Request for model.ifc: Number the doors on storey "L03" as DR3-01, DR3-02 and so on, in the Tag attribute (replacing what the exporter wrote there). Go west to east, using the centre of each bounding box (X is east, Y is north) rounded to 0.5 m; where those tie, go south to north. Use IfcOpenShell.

First a look at what the model holds.

```python
import ifcopenshell
import ifcopenshell.util.element
import ifcopenshell.util.placement

model = ifcopenshell.open("model.ifc")
print(model.schema)
storey = next(s for s in model.by_type("IfcBuildingStorey") if s.Name == "L03")
doors = [e for e in ifcopenshell.util.element.get_decomposition(storey) if e.is_a("IfcDoor")]
for e in sorted(doors, key=lambda e: e.id()):
    origin = ifcopenshell.util.placement.get_local_placement(e.ObjectPlacement)[:3, 3]
    print(e.id(), e.Tag, e.Name, origin.round(2) + 0.0, sep=" | ")
```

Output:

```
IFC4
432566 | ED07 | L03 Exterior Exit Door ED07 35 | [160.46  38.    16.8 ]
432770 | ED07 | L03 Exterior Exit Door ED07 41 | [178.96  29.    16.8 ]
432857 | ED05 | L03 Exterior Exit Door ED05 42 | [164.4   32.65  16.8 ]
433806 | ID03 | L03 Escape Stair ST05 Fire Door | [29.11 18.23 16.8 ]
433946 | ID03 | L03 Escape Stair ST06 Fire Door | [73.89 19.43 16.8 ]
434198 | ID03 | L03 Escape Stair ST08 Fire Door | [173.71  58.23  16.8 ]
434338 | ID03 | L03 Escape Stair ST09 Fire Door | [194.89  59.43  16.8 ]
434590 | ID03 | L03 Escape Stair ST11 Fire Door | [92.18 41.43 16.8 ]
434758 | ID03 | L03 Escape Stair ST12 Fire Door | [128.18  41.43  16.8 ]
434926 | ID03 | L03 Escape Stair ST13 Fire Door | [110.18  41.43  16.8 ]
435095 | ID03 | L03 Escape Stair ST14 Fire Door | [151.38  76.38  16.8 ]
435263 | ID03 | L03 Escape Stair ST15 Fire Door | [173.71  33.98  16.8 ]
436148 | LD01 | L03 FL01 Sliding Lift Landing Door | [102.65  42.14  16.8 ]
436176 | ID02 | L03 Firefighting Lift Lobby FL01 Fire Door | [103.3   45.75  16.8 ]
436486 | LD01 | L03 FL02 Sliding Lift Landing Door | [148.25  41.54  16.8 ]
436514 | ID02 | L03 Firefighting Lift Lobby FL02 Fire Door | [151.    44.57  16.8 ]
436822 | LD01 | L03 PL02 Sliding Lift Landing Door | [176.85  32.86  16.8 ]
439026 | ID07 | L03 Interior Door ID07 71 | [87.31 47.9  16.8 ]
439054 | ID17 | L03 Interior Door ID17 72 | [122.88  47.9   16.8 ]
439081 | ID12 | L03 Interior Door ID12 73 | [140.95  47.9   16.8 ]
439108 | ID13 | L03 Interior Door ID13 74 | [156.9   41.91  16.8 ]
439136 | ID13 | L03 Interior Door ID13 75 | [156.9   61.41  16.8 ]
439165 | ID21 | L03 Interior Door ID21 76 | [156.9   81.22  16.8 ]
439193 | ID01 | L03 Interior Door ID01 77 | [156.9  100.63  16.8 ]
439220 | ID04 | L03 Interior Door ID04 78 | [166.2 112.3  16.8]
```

```python
import ifcopenshell
import ifcopenshell.geom
import ifcopenshell.util.element
import ifcopenshell.util.shape

model = ifcopenshell.open("model.ifc")
settings = ifcopenshell.geom.settings()
settings.set("use-world-coords", True)


def centre(element):
    shape = ifcopenshell.geom.create_shape(settings, element)
    return ifcopenshell.util.shape.get_bbox_centroid(shape.geometry)


storey = next(s for s in model.by_type("IfcBuildingStorey") if s.Name == "L03")
doors = [e for e in ifcopenshell.util.element.get_decomposition(storey) if e.is_a("IfcDoor")]

# Insertion points can sit at a corner or the storey origin, so sort by the geometry (in metres).
centres = {e: centre(e) for e in doors}
doors.sort(key=lambda e: (round(centres[e][0] / 0.5), centres[e][1]))

for i, e in enumerate(doors, start=1):
    number = f"DR3-{i:02d}"
    e.Tag = number
    print(e.id(), number)

model.write("model_updated.ifc")
```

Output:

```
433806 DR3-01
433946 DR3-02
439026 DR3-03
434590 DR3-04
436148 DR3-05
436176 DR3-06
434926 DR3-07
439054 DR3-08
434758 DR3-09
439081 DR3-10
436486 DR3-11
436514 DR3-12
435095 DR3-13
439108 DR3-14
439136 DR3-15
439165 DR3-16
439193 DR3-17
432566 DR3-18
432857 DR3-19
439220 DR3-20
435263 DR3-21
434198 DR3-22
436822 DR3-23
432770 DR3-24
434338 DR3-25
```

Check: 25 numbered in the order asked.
